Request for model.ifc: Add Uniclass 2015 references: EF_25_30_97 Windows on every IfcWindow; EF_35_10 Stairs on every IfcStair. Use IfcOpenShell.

First a look at what the model holds.

```python
import ifcopenshell

model = ifcopenshell.open("model.ifc")
print(model.schema)
print("classifications:", [c.Name for c in model.by_type("IfcClassification")])
for ifc_class in ("IfcDoor", "IfcRoof", "IfcStair", "IfcWall", "IfcWindow"):
    print(ifc_class, len(model.by_type(ifc_class)))
```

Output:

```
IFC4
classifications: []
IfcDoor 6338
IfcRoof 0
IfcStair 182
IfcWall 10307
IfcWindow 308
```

```python
import ifcopenshell
import ifcopenshell.api.classification

model = ifcopenshell.open("model.ifc")

system = ifcopenshell.api.classification.add_classification(model, classification="Uniclass 2015")

codes = {
    "IfcWindow": ("EF_25_30_97", "Windows"),
    "IfcStair": ("EF_35_10", "Stairs"),
}
for ifc_class, (code, name) in codes.items():
    products = model.by_type(ifc_class)
    ifcopenshell.api.classification.add_reference(
        model, products=products, classification=system, identification=code, name=name
    )
    print(code, len(products))

model.write("model_v2.ifc")
```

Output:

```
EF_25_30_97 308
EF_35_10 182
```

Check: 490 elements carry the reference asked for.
